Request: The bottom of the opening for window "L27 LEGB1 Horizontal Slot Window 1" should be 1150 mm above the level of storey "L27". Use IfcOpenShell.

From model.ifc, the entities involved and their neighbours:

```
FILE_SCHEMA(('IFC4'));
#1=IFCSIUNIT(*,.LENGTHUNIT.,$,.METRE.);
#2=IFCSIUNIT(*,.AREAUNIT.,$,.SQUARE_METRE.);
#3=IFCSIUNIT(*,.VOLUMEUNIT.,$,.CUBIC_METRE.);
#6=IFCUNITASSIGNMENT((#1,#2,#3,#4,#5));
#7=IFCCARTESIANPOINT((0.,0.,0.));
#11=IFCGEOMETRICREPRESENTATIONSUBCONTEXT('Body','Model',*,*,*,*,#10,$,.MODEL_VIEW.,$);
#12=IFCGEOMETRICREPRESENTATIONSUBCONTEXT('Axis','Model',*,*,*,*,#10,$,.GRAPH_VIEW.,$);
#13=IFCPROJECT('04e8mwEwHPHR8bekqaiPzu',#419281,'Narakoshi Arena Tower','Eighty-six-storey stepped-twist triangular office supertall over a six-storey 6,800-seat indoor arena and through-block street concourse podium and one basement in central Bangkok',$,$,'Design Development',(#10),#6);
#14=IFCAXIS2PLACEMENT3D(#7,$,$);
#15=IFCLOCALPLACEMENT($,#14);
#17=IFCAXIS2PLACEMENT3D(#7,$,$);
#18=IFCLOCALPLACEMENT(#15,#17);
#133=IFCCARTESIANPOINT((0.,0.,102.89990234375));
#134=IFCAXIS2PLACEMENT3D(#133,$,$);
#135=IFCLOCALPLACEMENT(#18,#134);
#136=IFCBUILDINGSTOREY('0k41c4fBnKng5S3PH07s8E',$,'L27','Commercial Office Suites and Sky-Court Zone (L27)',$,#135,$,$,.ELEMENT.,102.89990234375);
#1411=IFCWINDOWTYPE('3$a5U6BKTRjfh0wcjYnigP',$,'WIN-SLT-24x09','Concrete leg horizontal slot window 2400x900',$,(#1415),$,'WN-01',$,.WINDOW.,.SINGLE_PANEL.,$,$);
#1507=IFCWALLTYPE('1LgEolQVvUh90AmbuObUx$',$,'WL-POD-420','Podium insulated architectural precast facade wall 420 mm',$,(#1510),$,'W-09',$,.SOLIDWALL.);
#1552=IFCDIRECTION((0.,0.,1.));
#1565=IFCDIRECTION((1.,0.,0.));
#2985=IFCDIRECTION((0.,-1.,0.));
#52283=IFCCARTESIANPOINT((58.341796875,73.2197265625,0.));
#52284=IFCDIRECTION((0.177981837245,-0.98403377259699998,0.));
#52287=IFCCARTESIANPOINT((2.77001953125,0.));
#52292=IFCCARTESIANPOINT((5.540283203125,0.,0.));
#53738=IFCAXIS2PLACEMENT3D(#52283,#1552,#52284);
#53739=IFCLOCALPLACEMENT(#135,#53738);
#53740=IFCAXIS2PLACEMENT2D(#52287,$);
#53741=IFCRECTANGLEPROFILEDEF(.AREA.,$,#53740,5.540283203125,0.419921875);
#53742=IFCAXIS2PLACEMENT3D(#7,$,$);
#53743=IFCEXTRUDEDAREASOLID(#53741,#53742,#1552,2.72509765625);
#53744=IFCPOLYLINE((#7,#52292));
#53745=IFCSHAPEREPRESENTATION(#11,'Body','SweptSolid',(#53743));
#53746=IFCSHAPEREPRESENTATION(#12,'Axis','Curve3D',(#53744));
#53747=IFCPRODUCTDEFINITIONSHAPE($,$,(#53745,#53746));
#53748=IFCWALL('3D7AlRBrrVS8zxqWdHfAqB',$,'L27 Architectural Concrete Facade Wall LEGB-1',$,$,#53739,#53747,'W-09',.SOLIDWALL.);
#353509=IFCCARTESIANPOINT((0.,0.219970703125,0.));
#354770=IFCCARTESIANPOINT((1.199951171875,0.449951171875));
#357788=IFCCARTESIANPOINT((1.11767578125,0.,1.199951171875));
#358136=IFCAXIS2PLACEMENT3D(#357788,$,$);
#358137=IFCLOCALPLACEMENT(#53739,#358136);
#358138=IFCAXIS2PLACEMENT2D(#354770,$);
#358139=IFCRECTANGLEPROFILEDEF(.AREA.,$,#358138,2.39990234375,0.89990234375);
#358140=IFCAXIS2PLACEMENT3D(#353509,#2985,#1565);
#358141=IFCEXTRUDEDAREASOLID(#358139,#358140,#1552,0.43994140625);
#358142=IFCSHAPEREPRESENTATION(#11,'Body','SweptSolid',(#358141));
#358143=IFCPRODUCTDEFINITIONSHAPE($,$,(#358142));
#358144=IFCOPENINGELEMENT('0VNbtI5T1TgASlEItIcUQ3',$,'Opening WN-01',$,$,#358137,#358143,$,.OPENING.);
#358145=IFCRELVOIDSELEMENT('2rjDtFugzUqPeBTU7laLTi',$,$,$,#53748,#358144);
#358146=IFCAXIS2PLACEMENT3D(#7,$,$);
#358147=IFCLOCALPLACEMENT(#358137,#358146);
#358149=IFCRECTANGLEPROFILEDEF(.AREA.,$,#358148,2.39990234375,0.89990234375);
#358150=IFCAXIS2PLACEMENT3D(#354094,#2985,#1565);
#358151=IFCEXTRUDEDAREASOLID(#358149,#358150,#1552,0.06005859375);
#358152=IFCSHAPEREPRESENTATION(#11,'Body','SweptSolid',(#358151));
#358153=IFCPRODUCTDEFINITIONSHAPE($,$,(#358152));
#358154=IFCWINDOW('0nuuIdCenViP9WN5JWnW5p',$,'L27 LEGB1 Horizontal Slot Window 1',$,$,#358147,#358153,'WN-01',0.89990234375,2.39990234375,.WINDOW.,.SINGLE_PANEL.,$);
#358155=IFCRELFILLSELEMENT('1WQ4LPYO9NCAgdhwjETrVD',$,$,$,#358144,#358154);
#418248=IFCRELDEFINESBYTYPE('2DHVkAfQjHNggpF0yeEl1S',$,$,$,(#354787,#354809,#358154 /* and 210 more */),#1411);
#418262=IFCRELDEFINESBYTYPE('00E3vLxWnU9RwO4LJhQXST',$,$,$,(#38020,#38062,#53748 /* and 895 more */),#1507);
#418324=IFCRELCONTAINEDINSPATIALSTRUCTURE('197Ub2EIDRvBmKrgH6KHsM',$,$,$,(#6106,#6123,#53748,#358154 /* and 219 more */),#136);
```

```python
import numpy as np
import ifcopenshell
import ifcopenshell.api.geometry
import ifcopenshell.geom
import ifcopenshell.util.element
import ifcopenshell.util.placement
import ifcopenshell.util.shape
import ifcopenshell.util.unit

model = ifcopenshell.open("model.ifc")
unit_scale = ifcopenshell.util.unit.calculate_unit_scale(model)

window = model.by_guid("0nuuIdCenViP9WN5JWnW5p")
opening = window.FillsVoids[0].RelatingOpeningElement
storey = ifcopenshell.util.element.get_container(window, ifc_class="IfcBuildingStorey")
level = ifcopenshell.util.placement.get_local_placement(storey.ObjectPlacement)[2, 3]

# The opening's origin need not be at the sill, so measure its lowest point.
shape = ifcopenshell.geom.create_shape(ifcopenshell.geom.settings(), opening)
bottom = ifcopenshell.util.shape.get_shape_bottom_elevation(shape, shape.geometry) / unit_scale
dz = level + 1.15 - bottom

shift = np.array([0.0, 0.0, dz])
# The window is placed relative to its opening, so it follows when the opening moves.
matrix = ifcopenshell.util.placement.get_local_placement(opening.ObjectPlacement)
matrix[:3, 3] += shift
ifcopenshell.api.geometry.edit_object_placement(
    model, product=opening, matrix=matrix, is_si=False, should_transform_children=True
)

print(f"moved by {dz * unit_scale:+.3f} m")

model.write("model_v2.ifc")
```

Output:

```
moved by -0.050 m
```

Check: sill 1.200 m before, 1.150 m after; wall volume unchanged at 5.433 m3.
